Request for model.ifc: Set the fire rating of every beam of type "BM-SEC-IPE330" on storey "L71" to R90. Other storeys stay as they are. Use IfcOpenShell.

First a look at what the model holds.

```python
import ifcopenshell
import ifcopenshell.util.element

model = ifcopenshell.open("model.ifc")
print(model.schema)
storey = next(s for s in model.by_type("IfcBuildingStorey") if s.Name == "L71")
beams = [e for e in ifcopenshell.util.element.get_decomposition(storey) if e.is_a("IfcBeam")]
seen = {}
for e in beams:
    element_type = ifcopenshell.util.element.get_type(e)
    key = (element_type.Name if element_type != e and element_type else None, ifcopenshell.util.element.get_pset(e, "Pset_BeamCommon", "FireRating"))
    seen[key] = seen.get(key, 0) + 1
for (name, value), count in sorted(seen.items(), key=str):
    print(count, "x", name, "|", value)
```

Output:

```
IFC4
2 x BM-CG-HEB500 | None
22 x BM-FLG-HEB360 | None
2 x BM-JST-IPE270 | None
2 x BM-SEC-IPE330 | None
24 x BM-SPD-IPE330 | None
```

```python
import ifcopenshell
import ifcopenshell.api.pset
import ifcopenshell.util.element

model = ifcopenshell.open("model.ifc")

storey = next(s for s in model.by_type("IfcBuildingStorey") if s.Name == "L71")
beams = [e for e in ifcopenshell.util.element.get_decomposition(storey) if e.is_a("IfcBeam")]

count = 0
for e in beams:
    element_type = ifcopenshell.util.element.get_type(e)
    if element_type in (None, e) or element_type.Name != "BM-SEC-IPE330":
        continue
    # add_pset returns the element's existing set when there is one.
    pset = ifcopenshell.api.pset.add_pset(model, product=e, name="Pset_BeamCommon")
    ifcopenshell.api.pset.edit_pset(model, pset=pset, properties={"FireRating": "R90"})
    count += 1

print(count, "beams updated")

model.write("model_rev.ifc")
```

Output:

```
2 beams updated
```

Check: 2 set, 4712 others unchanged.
